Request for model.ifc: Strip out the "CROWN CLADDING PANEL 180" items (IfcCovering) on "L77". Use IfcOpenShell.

First a look at what the model holds.

```python
import ifcopenshell
import ifcopenshell.util.element

model = ifcopenshell.open("model.ifc")
print(model.schema)
storey = next(s for s in model.by_type("IfcBuildingStorey") if s.Name == "L77")
coverings = [e for e in ifcopenshell.util.element.get_decomposition(storey) if e.is_a("IfcCovering")]
seen = {}
for e in coverings:
    element_type = ifcopenshell.util.element.get_type(e)
    name = element_type.Name if element_type not in (None, e) else None
    seen[name] = seen.get(name, 0) + 1
for name, count in sorted(seen.items(), key=str):
    print(count, "x", name)
```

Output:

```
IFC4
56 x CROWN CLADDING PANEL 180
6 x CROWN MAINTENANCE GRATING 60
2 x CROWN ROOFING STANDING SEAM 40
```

```python
import ifcopenshell
import ifcopenshell.api.root
import ifcopenshell.util.element

model = ifcopenshell.open("model.ifc")

storey = next(s for s in model.by_type("IfcBuildingStorey") if s.Name == "L77")
coverings = [e for e in ifcopenshell.util.element.get_decomposition(storey) if e.is_a("IfcCovering")]
targets = [e for e in coverings if (t := ifcopenshell.util.element.get_type(e)) not in (None, e) and t.Name == "CROWN CLADDING PANEL 180"]

for e in targets:
    ifcopenshell.api.root.remove_product(model, product=e)
print(len(targets), "removed")

model.write("model_rev.ifc")
```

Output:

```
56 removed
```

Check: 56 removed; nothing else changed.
